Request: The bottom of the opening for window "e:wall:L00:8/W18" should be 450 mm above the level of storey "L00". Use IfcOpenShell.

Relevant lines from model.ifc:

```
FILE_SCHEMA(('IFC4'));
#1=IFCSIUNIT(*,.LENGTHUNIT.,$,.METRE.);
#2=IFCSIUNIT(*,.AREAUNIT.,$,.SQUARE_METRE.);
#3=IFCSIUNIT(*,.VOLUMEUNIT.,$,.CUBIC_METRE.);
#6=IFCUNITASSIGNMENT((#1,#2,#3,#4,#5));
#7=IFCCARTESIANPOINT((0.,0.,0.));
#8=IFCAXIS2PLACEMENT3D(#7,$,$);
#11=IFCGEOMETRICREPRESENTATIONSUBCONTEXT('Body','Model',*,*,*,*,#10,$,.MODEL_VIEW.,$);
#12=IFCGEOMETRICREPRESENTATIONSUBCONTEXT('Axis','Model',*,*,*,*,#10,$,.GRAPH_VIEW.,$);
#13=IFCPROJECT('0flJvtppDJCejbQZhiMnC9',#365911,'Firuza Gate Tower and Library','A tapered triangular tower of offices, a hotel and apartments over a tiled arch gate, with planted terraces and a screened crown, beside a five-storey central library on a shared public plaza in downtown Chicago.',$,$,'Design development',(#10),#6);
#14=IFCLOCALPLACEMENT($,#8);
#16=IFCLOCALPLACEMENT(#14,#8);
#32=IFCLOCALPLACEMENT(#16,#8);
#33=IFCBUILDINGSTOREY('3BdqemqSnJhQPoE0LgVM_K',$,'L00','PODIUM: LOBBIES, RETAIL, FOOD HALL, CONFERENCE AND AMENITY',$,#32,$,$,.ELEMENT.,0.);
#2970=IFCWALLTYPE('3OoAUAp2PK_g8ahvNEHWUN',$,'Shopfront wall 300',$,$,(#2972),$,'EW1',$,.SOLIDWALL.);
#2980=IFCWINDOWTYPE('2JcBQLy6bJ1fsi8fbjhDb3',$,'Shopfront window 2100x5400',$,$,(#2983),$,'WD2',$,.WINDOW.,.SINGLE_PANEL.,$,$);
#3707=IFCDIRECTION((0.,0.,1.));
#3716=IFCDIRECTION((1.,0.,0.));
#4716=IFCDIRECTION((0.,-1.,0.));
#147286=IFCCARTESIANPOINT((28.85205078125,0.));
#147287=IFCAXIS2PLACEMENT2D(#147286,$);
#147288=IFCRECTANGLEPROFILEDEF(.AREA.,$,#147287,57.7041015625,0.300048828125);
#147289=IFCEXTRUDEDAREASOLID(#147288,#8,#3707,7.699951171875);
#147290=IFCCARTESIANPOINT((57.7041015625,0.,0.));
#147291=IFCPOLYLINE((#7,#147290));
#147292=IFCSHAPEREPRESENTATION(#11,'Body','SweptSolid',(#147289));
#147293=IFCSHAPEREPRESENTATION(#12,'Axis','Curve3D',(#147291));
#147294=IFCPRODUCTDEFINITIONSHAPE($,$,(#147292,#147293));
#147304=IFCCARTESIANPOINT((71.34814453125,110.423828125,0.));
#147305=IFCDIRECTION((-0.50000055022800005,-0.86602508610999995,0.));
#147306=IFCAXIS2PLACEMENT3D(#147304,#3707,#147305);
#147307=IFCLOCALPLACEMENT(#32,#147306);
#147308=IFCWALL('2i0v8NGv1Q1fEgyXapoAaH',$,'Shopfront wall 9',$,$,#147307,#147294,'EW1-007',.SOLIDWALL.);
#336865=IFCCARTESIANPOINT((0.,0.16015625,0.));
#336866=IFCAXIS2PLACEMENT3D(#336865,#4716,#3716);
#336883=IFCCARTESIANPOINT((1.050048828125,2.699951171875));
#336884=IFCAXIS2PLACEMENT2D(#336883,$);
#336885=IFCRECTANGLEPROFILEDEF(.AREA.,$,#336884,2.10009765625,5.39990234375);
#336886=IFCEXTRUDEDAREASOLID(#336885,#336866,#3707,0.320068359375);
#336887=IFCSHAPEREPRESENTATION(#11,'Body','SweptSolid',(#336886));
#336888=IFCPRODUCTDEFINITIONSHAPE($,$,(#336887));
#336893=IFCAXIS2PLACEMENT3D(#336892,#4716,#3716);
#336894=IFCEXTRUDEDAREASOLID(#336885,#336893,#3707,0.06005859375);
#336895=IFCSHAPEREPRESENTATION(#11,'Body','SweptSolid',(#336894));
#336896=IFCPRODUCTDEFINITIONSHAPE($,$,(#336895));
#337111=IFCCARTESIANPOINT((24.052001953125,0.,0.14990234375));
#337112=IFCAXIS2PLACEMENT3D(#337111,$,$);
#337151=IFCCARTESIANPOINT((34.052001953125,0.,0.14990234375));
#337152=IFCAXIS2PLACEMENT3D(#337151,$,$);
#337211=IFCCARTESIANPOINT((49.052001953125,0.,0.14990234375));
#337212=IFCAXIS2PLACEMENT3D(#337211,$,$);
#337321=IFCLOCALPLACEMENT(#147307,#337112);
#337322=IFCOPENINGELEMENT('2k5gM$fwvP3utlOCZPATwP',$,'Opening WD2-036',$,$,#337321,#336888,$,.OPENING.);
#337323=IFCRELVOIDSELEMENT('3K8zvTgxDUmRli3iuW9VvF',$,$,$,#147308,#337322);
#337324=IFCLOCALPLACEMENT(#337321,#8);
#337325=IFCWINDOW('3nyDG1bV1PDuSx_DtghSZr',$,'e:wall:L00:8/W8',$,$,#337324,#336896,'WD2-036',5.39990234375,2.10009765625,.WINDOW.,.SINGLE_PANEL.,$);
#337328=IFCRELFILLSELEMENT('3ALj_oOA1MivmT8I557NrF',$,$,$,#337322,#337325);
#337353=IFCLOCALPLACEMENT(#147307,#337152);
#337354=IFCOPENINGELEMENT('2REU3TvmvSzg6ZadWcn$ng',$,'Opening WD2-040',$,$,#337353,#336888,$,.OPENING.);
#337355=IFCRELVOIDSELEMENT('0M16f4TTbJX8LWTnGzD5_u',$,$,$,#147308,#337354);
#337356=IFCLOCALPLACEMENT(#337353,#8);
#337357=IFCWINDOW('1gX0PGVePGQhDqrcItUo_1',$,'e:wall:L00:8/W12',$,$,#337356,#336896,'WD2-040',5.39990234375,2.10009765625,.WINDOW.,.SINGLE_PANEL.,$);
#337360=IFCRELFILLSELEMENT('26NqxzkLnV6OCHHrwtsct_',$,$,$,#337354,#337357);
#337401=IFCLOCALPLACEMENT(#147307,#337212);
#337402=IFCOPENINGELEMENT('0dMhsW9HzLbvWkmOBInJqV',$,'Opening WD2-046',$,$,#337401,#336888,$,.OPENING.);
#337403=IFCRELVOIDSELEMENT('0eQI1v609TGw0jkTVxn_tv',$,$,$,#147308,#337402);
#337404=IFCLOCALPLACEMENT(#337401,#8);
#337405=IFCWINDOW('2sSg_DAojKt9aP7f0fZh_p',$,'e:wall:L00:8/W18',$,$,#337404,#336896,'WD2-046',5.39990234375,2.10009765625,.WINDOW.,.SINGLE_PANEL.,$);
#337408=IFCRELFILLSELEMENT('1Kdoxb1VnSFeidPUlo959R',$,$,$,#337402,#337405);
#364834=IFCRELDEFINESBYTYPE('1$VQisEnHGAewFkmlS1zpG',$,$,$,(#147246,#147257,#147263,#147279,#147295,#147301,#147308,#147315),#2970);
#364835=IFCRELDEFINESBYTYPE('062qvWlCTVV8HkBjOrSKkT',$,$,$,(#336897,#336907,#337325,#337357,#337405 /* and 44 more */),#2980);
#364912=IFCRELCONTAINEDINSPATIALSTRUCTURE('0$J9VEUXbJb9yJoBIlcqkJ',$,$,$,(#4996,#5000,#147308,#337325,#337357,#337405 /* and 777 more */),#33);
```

```python
import numpy as np
import ifcopenshell
import ifcopenshell.api.geometry
import ifcopenshell.geom
import ifcopenshell.util.element
import ifcopenshell.util.placement
import ifcopenshell.util.shape
import ifcopenshell.util.unit

model = ifcopenshell.open("model.ifc")
unit_scale = ifcopenshell.util.unit.calculate_unit_scale(model)

window = model.by_guid("2sSg_DAojKt9aP7f0fZh_p")
opening = window.FillsVoids[0].RelatingOpeningElement
storey = ifcopenshell.util.element.get_container(window, ifc_class="IfcBuildingStorey")
level = ifcopenshell.util.placement.get_local_placement(storey.ObjectPlacement)[2, 3]

# The opening's origin need not be at the sill, so measure its lowest point.
shape = ifcopenshell.geom.create_shape(ifcopenshell.geom.settings(), opening)
bottom = ifcopenshell.util.shape.get_shape_bottom_elevation(shape, shape.geometry) / unit_scale
dz = level + 0.45 / unit_scale - bottom

shift = np.array([0.0, 0.0, dz])
# The window is placed relative to its opening, so it follows when the opening moves.
matrix = ifcopenshell.util.placement.get_local_placement(opening.ObjectPlacement)
matrix[:3, 3] += shift
ifcopenshell.api.geometry.edit_object_placement(
    model, product=opening, matrix=matrix, is_si=False, should_transform_children=True
)

print(f"moved by {dz * unit_scale:+.3f} m")

model.write("model_edited.ifc")
```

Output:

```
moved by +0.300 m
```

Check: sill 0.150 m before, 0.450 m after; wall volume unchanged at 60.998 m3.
